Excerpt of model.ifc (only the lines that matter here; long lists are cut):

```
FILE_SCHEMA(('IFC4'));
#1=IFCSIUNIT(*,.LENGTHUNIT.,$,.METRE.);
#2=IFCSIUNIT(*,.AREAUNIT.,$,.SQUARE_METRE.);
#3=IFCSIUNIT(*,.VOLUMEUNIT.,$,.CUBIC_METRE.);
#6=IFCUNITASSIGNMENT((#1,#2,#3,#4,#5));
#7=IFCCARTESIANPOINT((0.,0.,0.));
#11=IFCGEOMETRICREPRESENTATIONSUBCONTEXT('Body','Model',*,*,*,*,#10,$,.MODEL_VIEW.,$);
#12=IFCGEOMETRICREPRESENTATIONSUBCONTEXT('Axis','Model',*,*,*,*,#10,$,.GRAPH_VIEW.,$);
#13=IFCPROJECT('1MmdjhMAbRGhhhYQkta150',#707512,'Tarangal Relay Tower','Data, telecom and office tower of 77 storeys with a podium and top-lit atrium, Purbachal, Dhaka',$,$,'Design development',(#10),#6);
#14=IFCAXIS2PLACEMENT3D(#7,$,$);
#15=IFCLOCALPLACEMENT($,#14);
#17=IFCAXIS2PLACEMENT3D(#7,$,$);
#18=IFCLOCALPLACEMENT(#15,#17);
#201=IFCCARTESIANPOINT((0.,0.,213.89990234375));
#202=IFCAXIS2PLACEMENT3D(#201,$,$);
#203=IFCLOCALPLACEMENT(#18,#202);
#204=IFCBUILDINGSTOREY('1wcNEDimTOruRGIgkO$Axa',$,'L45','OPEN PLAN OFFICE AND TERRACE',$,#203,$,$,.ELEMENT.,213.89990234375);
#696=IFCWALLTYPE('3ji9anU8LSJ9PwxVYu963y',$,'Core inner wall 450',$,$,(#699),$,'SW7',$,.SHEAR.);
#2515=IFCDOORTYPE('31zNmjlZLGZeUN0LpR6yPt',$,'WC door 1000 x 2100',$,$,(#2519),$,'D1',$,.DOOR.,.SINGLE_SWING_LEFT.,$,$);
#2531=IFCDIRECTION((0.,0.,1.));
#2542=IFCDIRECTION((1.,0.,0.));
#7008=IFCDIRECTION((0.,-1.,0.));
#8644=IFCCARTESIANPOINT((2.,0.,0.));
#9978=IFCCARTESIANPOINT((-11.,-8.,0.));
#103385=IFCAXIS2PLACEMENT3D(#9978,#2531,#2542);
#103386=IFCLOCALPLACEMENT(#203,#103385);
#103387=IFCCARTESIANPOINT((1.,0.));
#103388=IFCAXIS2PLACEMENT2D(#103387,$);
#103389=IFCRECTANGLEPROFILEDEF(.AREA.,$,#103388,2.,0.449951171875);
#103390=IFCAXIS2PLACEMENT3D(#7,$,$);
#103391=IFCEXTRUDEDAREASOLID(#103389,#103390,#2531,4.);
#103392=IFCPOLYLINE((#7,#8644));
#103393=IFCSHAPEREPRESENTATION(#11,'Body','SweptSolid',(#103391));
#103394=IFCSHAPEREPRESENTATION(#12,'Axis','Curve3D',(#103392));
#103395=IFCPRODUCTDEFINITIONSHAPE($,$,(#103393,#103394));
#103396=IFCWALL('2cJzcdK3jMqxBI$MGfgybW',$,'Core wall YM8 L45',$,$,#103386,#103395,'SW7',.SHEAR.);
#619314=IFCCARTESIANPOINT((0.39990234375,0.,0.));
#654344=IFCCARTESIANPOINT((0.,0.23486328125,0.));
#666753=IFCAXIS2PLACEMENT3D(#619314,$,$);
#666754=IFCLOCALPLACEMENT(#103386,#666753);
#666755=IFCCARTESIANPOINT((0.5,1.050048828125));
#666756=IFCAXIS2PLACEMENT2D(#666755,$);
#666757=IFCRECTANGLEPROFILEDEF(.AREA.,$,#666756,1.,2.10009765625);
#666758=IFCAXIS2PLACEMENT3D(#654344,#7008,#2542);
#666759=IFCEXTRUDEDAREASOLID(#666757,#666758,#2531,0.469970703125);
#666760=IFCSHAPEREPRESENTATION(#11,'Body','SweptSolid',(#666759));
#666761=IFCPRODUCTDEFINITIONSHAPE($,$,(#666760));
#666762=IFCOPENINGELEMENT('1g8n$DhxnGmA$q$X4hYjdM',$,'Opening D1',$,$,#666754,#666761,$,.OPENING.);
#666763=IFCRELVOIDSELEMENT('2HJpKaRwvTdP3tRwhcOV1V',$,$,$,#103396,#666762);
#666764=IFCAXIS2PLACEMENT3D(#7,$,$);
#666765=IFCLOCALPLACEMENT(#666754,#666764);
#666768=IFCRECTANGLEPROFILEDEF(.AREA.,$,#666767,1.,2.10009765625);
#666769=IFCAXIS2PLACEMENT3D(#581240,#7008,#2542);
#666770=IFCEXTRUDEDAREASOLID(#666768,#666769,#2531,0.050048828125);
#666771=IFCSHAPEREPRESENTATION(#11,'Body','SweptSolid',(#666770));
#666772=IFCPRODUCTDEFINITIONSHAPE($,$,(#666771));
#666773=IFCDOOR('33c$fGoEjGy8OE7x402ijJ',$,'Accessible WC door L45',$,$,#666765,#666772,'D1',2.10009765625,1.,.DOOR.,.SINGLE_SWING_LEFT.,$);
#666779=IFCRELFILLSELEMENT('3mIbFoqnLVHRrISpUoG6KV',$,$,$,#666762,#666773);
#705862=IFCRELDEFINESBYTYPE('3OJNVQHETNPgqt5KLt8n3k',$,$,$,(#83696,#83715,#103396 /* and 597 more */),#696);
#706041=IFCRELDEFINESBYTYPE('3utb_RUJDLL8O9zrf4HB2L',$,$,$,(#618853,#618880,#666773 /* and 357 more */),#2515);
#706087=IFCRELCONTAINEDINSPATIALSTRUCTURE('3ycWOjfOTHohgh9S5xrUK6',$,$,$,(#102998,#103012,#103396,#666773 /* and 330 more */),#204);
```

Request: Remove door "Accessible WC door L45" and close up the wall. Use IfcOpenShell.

```python
import ifcopenshell
import ifcopenshell.api.feature
import ifcopenshell.api.root
import ifcopenshell.geom
import ifcopenshell.util.shape

model = ifcopenshell.open("model.ifc")
settings = ifcopenshell.geom.settings()


def volume(element):
    """Net volume in cubic metres, openings subtracted."""
    shape = ifcopenshell.geom.create_shape(settings, element)
    return ifcopenshell.util.shape.get_volume(shape.geometry)


door = model.by_guid("33c$fGoEjGy8OE7x402ijJ")
opening = door.FillsVoids[0].RelatingOpeningElement
wall = opening.VoidsElements[0].RelatingBuildingElement
before = volume(wall)

ifcopenshell.api.root.remove_product(model, product=door)
ifcopenshell.api.feature.remove_feature(model, feature=opening)

after = volume(wall)

print(f"wall volume {before:.3f} -> {after:.3f} m3")

model.write("model_updated.ifc")
```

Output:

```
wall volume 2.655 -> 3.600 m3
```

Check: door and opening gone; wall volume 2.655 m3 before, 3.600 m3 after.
